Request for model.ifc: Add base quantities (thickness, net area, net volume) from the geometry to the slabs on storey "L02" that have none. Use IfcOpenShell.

First a look at what the model holds.

```python
import ifcopenshell
import ifcopenshell.util.element
import ifcopenshell.util.unit

model = ifcopenshell.open("model.ifc")
print(model.schema)
for unit_type in ("LENGTHUNIT", "AREAUNIT", "VOLUMEUNIT"):
    print(unit_type, ifcopenshell.util.unit.calculate_unit_scale(model, unit_type))
storey = next(s for s in model.by_type("IfcBuildingStorey") if s.Name == "L02")
slabs = [e for e in ifcopenshell.util.element.get_decomposition(storey) if e.is_a("IfcSlab")]
for e in sorted(slabs, key=lambda e: e.id()):
    print(e.id(), e.is_a(), e.Name, list(ifcopenshell.util.element.get_psets(e, qtos_only=True)), sep=" | ")
```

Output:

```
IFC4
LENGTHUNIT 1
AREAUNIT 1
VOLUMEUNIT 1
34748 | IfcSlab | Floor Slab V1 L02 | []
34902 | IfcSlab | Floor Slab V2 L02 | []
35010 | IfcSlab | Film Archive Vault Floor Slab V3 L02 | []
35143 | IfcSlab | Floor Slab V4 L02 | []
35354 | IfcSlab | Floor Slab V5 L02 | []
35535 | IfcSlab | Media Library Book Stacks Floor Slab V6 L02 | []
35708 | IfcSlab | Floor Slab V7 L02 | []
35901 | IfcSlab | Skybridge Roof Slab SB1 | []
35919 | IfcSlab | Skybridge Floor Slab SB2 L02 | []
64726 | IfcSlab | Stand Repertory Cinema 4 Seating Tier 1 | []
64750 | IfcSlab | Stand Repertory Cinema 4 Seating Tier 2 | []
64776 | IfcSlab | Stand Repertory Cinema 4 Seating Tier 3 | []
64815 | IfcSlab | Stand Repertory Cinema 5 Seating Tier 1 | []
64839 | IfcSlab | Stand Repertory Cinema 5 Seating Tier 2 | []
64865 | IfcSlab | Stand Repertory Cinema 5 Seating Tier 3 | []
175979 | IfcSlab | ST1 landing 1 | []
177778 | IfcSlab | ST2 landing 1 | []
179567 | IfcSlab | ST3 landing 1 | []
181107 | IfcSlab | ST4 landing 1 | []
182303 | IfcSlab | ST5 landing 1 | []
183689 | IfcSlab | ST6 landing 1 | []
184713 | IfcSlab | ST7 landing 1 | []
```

```python
import ifcopenshell
import ifcopenshell.api.pset
import ifcopenshell.geom
import ifcopenshell.util.element
import ifcopenshell.util.shape
import ifcopenshell.util.unit

model = ifcopenshell.open("model.ifc")
unit_scale = ifcopenshell.util.unit.calculate_unit_scale(model)
area_scale = ifcopenshell.util.unit.calculate_unit_scale(model, "AREAUNIT")
volume_scale = ifcopenshell.util.unit.calculate_unit_scale(model, "VOLUMEUNIT")
settings = ifcopenshell.geom.settings()

storey = next(s for s in model.by_type("IfcBuildingStorey") if s.Name == "L02")
slabs = [e for e in ifcopenshell.util.element.get_decomposition(storey) if e.is_a("IfcSlab")]

for e in sorted(slabs, key=lambda e: e.id()):
    if ifcopenshell.util.element.get_psets(e, qtos_only=True, should_inherit=False):
        continue
    # Geometry comes back in metres, in the element's own axes.
    shape = ifcopenshell.geom.create_shape(settings, e)
    values = {
        "Width": ifcopenshell.util.shape.get_z(shape.geometry) / unit_scale,
        "NetArea": ifcopenshell.util.shape.get_footprint_area(shape.geometry) / area_scale,
        "NetVolume": ifcopenshell.util.shape.get_volume(shape.geometry) / volume_scale,
    }
    qto = ifcopenshell.api.pset.add_qto(model, product=e, name="Qto_SlabBaseQuantities")
    ifcopenshell.api.pset.edit_qto(model, qto=qto, properties=values)
    print(e.id(), {k: round(v, 3) for k, v in values.items()})

model.write("model_rev.ifc")
```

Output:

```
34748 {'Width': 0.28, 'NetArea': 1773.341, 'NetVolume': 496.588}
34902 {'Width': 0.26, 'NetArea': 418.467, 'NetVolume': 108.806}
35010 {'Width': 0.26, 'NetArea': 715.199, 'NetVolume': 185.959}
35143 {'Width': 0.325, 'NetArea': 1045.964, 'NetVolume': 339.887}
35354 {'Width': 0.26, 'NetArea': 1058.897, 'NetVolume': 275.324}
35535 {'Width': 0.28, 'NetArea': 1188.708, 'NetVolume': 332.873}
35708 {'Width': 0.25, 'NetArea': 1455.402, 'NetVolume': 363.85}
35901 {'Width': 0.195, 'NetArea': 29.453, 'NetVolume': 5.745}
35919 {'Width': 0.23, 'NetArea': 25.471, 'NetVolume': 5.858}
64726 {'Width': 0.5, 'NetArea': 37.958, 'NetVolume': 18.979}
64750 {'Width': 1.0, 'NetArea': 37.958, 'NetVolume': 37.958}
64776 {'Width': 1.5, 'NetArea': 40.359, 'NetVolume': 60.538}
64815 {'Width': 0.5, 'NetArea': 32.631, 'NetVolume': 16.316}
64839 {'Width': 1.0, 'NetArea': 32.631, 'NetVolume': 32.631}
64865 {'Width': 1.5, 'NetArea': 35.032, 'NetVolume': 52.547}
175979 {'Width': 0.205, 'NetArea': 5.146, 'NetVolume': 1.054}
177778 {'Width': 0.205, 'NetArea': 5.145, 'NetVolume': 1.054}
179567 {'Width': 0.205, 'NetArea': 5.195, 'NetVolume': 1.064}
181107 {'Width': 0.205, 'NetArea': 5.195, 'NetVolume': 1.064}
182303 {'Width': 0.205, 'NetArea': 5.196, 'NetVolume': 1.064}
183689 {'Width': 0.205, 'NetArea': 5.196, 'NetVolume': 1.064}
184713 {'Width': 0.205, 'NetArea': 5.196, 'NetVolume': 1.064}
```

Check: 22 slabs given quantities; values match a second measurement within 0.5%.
